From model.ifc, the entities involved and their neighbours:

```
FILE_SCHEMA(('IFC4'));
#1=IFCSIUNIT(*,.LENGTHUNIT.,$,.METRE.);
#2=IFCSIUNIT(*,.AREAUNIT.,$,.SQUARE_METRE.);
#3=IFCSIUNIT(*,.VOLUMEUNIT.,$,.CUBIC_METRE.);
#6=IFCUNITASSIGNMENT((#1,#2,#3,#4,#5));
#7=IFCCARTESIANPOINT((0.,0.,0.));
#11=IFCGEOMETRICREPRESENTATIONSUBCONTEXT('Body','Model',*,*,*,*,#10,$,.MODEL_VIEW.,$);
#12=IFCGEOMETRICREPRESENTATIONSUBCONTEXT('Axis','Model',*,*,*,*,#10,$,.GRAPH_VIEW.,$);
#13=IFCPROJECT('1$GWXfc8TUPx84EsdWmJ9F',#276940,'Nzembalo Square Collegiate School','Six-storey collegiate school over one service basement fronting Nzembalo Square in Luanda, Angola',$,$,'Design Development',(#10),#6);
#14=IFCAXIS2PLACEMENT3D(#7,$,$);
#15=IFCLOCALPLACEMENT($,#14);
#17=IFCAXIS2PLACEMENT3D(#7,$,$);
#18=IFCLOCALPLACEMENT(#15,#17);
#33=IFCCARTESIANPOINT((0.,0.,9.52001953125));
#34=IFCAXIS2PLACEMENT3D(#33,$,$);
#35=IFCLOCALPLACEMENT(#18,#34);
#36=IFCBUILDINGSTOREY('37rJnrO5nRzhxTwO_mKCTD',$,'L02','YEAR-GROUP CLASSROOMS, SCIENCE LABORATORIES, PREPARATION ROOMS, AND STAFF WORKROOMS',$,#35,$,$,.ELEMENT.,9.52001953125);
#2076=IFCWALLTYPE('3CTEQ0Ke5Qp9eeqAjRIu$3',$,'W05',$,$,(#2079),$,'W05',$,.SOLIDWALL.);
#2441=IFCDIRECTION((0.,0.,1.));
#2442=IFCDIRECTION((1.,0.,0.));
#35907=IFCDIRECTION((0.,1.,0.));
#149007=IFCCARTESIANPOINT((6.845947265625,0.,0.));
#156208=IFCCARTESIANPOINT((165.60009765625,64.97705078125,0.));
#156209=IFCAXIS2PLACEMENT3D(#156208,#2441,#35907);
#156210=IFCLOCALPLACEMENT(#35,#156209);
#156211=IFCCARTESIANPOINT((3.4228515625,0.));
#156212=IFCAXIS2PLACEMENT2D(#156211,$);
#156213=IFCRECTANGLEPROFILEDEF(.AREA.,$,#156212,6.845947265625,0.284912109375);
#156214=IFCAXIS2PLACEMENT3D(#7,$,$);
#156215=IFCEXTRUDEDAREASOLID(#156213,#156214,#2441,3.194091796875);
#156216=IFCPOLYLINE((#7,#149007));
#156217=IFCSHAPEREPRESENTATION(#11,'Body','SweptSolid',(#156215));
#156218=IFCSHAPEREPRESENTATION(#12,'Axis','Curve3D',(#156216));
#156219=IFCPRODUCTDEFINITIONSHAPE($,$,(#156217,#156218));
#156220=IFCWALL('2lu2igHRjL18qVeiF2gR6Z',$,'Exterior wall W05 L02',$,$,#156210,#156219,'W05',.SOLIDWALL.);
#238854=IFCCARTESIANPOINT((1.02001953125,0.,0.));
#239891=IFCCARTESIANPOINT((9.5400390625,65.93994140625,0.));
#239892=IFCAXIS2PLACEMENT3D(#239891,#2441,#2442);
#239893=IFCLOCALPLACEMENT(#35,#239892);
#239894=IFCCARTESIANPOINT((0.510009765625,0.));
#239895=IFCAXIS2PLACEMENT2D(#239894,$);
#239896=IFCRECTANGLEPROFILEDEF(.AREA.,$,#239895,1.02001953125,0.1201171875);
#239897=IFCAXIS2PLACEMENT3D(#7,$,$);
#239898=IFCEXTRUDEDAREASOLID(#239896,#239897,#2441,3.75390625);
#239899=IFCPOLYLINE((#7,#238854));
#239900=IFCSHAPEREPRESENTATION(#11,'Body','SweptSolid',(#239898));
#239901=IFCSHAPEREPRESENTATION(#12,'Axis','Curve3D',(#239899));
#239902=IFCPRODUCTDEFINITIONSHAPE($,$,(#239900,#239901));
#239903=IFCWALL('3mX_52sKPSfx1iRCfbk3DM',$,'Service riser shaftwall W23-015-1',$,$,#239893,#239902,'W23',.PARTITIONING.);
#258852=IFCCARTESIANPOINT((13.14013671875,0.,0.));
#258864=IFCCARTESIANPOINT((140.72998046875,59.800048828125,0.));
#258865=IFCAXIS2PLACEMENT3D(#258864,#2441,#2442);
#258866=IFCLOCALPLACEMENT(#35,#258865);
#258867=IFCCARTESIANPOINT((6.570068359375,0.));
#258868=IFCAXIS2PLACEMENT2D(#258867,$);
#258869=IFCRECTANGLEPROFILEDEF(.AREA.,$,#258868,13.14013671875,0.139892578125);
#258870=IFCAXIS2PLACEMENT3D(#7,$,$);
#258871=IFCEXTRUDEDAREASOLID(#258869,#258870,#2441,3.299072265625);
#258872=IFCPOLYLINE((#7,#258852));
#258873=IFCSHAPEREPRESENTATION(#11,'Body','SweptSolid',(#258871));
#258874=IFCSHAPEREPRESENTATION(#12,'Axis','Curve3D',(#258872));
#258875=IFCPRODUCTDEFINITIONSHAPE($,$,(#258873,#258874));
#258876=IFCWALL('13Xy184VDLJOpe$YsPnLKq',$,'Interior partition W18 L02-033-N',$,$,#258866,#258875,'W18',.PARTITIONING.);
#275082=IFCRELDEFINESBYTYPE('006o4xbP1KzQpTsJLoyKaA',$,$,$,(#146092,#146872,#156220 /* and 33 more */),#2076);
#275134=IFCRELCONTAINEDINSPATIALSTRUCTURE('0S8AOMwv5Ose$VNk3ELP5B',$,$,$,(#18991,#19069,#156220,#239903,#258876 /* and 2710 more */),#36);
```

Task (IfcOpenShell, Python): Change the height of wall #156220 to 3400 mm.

```python
import ifcopenshell
import ifcopenshell.geom
import ifcopenshell.util.representation
import ifcopenshell.util.shape

model = ifcopenshell.open("model.ifc")
settings = ifcopenshell.geom.settings()


def volume(element):
    """Net volume in cubic metres, openings subtracted."""
    shape = ifcopenshell.geom.create_shape(settings, element)
    return ifcopenshell.util.shape.get_volume(shape.geometry)


wall = model.by_id(156220)
before = volume(wall)

body = ifcopenshell.util.representation.get_representation(wall, "Model", "Body")
solid = body.Items[0]
old_height = solid.Depth
solid.Depth = 3.4
after = volume(wall)

print(f"height {old_height:g} -> {solid.Depth:g}, volume {before:.3f} -> {after:.3f} m3")

model.write("model_v2.ifc")
```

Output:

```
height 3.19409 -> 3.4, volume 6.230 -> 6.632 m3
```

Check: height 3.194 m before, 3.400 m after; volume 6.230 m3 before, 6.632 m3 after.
